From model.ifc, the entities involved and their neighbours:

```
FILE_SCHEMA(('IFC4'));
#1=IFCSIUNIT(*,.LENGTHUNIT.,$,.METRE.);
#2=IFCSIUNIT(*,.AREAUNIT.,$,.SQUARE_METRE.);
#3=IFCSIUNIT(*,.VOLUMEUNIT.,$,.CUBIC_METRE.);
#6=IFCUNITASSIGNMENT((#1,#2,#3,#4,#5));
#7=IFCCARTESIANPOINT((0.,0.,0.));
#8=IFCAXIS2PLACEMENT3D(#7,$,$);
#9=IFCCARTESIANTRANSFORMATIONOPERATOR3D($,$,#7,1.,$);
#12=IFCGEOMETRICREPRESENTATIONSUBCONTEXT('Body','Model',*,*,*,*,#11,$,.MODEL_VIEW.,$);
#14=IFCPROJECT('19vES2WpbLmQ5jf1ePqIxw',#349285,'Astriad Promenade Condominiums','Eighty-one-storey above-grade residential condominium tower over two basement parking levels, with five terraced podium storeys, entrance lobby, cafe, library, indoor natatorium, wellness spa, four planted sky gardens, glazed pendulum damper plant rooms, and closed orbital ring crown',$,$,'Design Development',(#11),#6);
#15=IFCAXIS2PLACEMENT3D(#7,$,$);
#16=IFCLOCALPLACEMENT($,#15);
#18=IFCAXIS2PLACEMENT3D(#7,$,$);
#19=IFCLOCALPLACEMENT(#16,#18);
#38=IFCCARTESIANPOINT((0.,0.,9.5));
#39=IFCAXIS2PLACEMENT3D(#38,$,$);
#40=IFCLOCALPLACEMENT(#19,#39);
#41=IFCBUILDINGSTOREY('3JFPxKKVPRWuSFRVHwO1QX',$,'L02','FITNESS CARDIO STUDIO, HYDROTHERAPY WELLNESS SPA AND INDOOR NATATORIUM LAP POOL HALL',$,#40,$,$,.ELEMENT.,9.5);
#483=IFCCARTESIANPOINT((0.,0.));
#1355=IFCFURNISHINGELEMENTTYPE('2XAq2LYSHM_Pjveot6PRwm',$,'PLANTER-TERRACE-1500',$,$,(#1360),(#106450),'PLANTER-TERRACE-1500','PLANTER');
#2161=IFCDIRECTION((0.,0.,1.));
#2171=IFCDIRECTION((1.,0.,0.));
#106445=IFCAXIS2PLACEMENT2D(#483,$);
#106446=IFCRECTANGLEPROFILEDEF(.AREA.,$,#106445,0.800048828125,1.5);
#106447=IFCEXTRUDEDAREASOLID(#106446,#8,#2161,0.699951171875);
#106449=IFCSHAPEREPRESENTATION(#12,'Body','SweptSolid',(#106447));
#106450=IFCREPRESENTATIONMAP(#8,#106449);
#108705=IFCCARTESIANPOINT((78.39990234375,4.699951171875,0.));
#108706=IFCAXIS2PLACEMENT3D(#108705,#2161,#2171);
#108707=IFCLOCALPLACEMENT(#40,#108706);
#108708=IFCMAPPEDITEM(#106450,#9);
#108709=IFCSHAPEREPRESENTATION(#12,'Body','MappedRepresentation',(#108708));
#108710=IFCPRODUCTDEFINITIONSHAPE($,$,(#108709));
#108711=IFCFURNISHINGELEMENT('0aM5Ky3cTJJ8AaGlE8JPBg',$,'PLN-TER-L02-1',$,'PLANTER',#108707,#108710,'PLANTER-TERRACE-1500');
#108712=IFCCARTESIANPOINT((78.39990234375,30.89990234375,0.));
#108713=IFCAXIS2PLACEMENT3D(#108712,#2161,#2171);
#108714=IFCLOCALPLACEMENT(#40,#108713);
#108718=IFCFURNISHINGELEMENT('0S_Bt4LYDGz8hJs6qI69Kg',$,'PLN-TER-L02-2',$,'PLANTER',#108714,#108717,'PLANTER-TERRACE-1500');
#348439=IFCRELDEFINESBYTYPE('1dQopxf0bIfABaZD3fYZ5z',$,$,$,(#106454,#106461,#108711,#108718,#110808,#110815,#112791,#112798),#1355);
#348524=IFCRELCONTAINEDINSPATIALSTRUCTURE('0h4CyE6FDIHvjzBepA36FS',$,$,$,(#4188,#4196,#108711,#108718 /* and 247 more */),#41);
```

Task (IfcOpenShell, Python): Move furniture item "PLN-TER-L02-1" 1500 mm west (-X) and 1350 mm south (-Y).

```python
import ifcopenshell
import ifcopenshell.api.geometry
import ifcopenshell.util.placement
import ifcopenshell.util.unit

model = ifcopenshell.open("model.ifc")
unit_scale = ifcopenshell.util.unit.calculate_unit_scale(model)

item = model.by_guid("0aM5Ky3cTJJ8AaGlE8JPBg")
matrix = ifcopenshell.util.placement.get_local_placement(item.ObjectPlacement)
matrix[0, 3] -= 1.5 / unit_scale
matrix[1, 3] -= 1.35 / unit_scale
ifcopenshell.api.geometry.edit_object_placement(model, product=item, matrix=matrix, is_si=False)

print(ifcopenshell.util.placement.get_local_placement(item.ObjectPlacement).round(3) + 0.0)

model.write("model_v2.ifc")
```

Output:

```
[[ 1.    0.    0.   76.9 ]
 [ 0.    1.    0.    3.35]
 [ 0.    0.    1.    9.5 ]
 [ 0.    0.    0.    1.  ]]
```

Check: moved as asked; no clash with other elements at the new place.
